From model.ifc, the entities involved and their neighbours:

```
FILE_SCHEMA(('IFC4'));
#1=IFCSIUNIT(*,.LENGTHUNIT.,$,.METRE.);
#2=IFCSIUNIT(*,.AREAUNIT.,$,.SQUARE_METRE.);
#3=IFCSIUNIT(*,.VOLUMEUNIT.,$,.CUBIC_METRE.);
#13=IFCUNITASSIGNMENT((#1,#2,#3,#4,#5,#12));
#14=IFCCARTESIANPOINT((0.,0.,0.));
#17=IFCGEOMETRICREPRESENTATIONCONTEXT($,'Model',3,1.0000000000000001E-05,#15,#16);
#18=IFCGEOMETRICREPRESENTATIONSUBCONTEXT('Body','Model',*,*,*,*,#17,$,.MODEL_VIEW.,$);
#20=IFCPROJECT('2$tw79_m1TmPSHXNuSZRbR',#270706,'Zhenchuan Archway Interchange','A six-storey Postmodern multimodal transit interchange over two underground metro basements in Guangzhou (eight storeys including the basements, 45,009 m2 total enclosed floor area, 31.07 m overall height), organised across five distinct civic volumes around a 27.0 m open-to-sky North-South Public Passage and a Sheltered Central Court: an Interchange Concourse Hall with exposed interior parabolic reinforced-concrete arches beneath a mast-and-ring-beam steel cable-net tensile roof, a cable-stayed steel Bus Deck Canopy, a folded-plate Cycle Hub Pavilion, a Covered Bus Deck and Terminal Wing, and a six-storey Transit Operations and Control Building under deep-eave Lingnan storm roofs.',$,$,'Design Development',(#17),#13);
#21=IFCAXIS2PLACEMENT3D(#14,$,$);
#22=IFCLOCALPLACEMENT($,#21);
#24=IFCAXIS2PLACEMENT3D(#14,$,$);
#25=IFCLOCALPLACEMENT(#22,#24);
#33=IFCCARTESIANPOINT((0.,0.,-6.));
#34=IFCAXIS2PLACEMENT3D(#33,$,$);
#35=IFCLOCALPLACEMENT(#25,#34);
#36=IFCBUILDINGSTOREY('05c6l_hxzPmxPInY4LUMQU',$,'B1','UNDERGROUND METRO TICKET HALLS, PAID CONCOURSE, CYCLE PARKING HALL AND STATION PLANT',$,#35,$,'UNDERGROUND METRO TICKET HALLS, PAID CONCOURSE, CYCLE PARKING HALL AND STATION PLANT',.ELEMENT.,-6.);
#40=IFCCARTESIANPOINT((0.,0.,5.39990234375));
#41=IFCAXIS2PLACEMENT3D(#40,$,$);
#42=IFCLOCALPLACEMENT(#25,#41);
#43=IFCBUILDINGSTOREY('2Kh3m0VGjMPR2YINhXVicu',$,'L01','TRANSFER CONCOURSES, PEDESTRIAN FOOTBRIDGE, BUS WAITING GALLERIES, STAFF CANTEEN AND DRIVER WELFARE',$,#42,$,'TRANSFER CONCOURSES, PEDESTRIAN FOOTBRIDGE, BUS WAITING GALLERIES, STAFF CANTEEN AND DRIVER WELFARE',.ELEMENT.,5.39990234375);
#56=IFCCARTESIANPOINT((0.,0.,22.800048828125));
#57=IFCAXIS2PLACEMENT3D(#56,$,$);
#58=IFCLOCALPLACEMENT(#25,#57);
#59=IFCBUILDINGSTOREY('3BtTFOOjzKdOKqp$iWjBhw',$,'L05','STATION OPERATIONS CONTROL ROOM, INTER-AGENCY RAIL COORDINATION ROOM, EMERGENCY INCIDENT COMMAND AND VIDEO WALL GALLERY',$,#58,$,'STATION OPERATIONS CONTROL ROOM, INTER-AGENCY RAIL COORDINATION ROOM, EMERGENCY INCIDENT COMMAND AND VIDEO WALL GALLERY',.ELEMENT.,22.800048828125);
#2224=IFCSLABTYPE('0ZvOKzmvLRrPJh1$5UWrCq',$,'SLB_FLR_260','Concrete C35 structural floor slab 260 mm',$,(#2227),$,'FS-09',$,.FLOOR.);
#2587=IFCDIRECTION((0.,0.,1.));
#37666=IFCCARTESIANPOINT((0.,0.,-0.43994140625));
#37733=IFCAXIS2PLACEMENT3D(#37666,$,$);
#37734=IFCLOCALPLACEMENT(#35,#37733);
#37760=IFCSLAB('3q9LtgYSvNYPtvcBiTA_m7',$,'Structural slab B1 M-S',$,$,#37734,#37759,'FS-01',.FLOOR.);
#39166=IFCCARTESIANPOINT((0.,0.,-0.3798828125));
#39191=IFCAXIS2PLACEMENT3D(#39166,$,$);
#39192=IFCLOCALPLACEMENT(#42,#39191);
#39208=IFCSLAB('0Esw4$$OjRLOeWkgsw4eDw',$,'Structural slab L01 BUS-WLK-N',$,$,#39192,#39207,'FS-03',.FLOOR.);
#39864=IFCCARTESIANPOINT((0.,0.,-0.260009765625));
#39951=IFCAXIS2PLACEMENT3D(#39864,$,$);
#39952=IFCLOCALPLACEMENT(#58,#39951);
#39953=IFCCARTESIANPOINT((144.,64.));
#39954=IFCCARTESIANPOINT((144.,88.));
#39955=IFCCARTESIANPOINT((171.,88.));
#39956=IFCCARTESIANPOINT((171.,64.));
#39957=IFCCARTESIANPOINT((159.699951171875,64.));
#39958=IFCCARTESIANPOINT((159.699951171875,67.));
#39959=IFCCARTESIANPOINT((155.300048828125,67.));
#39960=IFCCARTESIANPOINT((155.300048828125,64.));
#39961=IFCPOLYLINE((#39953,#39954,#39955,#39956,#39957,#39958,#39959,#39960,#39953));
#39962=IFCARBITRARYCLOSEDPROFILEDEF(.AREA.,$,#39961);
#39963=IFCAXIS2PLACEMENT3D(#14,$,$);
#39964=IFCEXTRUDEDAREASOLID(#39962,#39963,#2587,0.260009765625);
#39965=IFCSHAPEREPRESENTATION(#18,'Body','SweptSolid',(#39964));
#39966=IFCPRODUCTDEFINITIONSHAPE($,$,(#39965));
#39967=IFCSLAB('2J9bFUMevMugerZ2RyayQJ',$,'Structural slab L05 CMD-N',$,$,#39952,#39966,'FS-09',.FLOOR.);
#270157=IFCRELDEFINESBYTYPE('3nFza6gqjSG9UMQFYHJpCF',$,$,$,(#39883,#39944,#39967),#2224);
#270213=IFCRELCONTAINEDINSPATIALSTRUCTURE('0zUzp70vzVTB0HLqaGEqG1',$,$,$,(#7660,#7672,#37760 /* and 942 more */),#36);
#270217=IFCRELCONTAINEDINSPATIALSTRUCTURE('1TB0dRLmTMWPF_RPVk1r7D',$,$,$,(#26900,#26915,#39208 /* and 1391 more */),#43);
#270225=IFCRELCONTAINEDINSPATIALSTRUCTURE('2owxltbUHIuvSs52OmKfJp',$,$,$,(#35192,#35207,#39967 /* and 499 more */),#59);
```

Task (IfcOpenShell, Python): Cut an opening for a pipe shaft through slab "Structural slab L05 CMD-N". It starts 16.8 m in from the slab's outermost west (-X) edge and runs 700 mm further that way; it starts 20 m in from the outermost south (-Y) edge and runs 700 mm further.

```python
import numpy as np
import ifcopenshell
import ifcopenshell.api.feature
import ifcopenshell.api.geometry
import ifcopenshell.api.root
import ifcopenshell.geom
import ifcopenshell.util.placement
import ifcopenshell.util.representation
import ifcopenshell.util.shape
import ifcopenshell.util.unit

model = ifcopenshell.open("model.ifc")
unit_scale = ifcopenshell.util.unit.calculate_unit_scale(model)
settings = ifcopenshell.geom.settings()


def volume(element):
    """Net volume in cubic metres, openings subtracted."""
    shape = ifcopenshell.geom.create_shape(settings, element)
    return ifcopenshell.util.shape.get_volume(shape.geometry)


slab = model.by_id(39967)
before = volume(slab)

# Extent in the slab's own axes, in metres. The edges named are its -X and -Y sides.
slab_shape = ifcopenshell.geom.create_shape(settings, slab)
vertices = ifcopenshell.util.shape.get_vertices(slab_shape.geometry)
x_min, y_min, bottom = vertices.min(axis=0)
top = vertices[:, 2].max()

opening = ifcopenshell.api.root.create_entity(model, ifc_class="IfcOpeningElement", name="Pipe shaft opening", predefined_type="OPENING")
context = ifcopenshell.util.representation.get_context(model, "Model", "Body", "MODEL_VIEW")
width, depth = 0.7, 0.7
outline = [(0.0, 0.0), (width, 0.0), (width, depth), (0.0, depth), (0.0, 0.0)]
# Overshoot both faces by 50 mm so the cut is clean.
shape = ifcopenshell.api.geometry.add_slab_representation(
    model, context=context, depth=top - bottom + 0.1, polyline=outline
)
ifcopenshell.api.geometry.assign_representation(model, product=opening, representation=shape)

matrix = ifcopenshell.util.placement.get_local_placement(slab.ObjectPlacement)
matrix[:, 3] = matrix @ np.append(np.array([x_min + 16.8, y_min + 20, bottom - 0.05]) / unit_scale, 1.0)
ifcopenshell.api.geometry.edit_object_placement(model, product=opening, matrix=matrix, is_si=False)
ifcopenshell.api.feature.add_feature(model, feature=opening, element=slab)

after = volume(slab)

print(f"slab volume {before:.3f} -> {after:.3f} m3")

model.write("model_updated.ifc")
```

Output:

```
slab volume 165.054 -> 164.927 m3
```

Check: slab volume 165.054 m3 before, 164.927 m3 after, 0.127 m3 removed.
